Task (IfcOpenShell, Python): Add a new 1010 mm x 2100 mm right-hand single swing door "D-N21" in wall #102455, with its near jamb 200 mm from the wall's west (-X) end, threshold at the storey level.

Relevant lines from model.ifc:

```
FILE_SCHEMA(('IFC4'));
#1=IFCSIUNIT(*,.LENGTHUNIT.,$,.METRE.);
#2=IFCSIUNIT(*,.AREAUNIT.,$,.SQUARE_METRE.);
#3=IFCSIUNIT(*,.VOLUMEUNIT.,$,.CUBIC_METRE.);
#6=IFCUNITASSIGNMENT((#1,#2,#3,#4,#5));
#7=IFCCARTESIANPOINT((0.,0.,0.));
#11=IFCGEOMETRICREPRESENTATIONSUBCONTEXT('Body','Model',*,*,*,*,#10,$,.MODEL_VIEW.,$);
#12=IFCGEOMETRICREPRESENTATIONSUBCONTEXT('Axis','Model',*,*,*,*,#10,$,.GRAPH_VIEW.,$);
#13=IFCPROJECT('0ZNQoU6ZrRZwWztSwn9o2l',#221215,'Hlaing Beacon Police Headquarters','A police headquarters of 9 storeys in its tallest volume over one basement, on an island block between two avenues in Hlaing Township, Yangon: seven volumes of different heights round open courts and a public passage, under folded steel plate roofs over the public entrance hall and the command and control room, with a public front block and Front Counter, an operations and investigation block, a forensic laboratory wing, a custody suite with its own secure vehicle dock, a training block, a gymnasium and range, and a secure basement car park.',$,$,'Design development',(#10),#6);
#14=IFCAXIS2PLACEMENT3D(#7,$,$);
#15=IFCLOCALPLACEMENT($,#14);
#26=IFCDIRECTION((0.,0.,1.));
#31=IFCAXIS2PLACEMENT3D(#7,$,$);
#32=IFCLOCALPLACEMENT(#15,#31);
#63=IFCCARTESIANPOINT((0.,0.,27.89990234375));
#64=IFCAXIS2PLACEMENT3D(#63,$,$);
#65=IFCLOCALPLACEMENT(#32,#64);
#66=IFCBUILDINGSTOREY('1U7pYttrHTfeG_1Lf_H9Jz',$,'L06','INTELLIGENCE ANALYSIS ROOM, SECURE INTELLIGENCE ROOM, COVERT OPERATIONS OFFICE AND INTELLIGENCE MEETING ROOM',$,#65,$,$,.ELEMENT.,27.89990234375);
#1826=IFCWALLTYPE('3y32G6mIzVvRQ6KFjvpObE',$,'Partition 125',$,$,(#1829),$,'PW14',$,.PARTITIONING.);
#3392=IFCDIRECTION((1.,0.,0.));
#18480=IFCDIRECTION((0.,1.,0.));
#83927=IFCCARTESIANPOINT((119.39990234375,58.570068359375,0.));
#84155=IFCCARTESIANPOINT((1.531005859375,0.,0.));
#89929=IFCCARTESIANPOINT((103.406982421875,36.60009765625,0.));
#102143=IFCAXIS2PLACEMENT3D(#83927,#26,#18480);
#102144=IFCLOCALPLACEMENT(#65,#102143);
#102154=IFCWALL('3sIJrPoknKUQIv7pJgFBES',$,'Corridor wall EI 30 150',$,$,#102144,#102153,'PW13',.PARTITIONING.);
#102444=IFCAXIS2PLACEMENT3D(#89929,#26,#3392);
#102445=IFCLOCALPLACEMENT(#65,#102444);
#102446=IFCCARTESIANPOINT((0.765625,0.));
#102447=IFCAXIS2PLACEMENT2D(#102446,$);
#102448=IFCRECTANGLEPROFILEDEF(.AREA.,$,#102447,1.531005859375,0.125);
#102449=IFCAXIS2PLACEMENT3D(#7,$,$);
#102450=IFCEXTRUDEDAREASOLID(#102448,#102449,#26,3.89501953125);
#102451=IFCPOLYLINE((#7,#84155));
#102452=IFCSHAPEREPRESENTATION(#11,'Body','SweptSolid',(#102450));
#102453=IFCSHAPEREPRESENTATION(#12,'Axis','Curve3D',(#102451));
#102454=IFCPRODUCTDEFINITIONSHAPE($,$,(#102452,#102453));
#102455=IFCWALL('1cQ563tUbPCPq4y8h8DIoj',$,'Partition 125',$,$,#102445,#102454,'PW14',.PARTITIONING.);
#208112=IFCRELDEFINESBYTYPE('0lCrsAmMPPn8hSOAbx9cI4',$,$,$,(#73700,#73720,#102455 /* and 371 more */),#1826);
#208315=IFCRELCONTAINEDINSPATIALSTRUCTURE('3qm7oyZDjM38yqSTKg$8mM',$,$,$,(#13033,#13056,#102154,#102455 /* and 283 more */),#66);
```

```python
import numpy as np
import ifcopenshell
import ifcopenshell.api.feature
import ifcopenshell.api.geometry
import ifcopenshell.api.root
import ifcopenshell.api.spatial
import ifcopenshell.geom
import ifcopenshell.util.element
import ifcopenshell.util.placement
import ifcopenshell.util.representation
import ifcopenshell.util.shape
import ifcopenshell.util.unit

model = ifcopenshell.open("model.ifc")
unit_scale = ifcopenshell.util.unit.calculate_unit_scale(model)
settings = ifcopenshell.geom.settings()


def volume(element):
    """Net volume in cubic metres, openings subtracted."""
    shape = ifcopenshell.geom.create_shape(settings, element)
    return ifcopenshell.util.shape.get_volume(shape.geometry)


wall = model.by_id(102455)
storey = ifcopenshell.util.element.get_container(wall, ifc_class="IfcBuildingStorey")
context = ifcopenshell.util.representation.get_context(model, "Model", "Body", "MODEL_VIEW")
before = volume(wall)

width, height, from_end, sill = 1.01, 2.1, 0.2, 0.0  # metres

# The wall runs along its own X axis, and the end named is its -X end.
wall_shape = ifcopenshell.geom.create_shape(settings, wall)
x, y, z = ifcopenshell.util.shape.get_vertices(wall_shape.geometry).T
start = x.min() + from_end
face, thickness = float(y.min()), float(y.max() - y.min())
wall_matrix = ifcopenshell.util.placement.get_local_placement(wall.ObjectPlacement)
level = ifcopenshell.util.placement.get_local_placement(storey.ObjectPlacement)[2, 3]


def in_wall(x, y):
    """Placement at x, y metres in the wall's axes, at sill height."""
    matrix = wall_matrix.copy()
    matrix[:, 3] = wall_matrix @ np.array([x / unit_scale, y / unit_scale, 0.0, 1.0])
    matrix[2, 3] = level + sill / unit_scale
    return matrix


# Opening: a box that overshoots both wall faces by 50 mm.
opening = ifcopenshell.api.root.create_entity(model, ifc_class="IfcOpeningElement", predefined_type="OPENING")
box = ifcopenshell.api.geometry.add_wall_representation(
    model, context=context, length=width, height=height, thickness=thickness + 0.1
)
ifcopenshell.api.geometry.assign_representation(model, product=opening, representation=box)
ifcopenshell.api.geometry.edit_object_placement(model, product=opening, matrix=in_wall(start, face - 0.05), is_si=False)
ifcopenshell.api.feature.add_feature(model, feature=opening, element=wall)

door = ifcopenshell.api.root.create_entity(model, ifc_class="IfcDoor", name="D-N21", predefined_type="DOOR")
door.OverallWidth, door.OverallHeight = width / unit_scale, height / unit_scale
door.OperationType = "SINGLE_SWING_RIGHT"
body = ifcopenshell.api.geometry.add_door_representation(
    model,
    context=context,
    overall_width=door.OverallWidth,
    overall_height=door.OverallHeight,
    operation_type="SINGLE_SWING_RIGHT",
    lining_properties={"LiningDepth": thickness / unit_scale, "ThresholdDepth": thickness / unit_scale},
)
ifcopenshell.api.geometry.assign_representation(model, product=door, representation=body)
ifcopenshell.api.spatial.assign_container(model, products=[door], relating_structure=storey)
ifcopenshell.api.feature.add_filling(model, opening=opening, element=door)

# The lining spans the wall, so the door starts at the wall face.
ifcopenshell.api.geometry.edit_object_placement(model, product=door, matrix=in_wall(start, face), is_si=False)

after = volume(wall)

print(f"wall volume {before:.3f} -> {after:.3f} m3")

model.write("model_rev.ifc")
```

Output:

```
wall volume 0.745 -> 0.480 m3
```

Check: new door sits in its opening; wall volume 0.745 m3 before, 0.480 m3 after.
